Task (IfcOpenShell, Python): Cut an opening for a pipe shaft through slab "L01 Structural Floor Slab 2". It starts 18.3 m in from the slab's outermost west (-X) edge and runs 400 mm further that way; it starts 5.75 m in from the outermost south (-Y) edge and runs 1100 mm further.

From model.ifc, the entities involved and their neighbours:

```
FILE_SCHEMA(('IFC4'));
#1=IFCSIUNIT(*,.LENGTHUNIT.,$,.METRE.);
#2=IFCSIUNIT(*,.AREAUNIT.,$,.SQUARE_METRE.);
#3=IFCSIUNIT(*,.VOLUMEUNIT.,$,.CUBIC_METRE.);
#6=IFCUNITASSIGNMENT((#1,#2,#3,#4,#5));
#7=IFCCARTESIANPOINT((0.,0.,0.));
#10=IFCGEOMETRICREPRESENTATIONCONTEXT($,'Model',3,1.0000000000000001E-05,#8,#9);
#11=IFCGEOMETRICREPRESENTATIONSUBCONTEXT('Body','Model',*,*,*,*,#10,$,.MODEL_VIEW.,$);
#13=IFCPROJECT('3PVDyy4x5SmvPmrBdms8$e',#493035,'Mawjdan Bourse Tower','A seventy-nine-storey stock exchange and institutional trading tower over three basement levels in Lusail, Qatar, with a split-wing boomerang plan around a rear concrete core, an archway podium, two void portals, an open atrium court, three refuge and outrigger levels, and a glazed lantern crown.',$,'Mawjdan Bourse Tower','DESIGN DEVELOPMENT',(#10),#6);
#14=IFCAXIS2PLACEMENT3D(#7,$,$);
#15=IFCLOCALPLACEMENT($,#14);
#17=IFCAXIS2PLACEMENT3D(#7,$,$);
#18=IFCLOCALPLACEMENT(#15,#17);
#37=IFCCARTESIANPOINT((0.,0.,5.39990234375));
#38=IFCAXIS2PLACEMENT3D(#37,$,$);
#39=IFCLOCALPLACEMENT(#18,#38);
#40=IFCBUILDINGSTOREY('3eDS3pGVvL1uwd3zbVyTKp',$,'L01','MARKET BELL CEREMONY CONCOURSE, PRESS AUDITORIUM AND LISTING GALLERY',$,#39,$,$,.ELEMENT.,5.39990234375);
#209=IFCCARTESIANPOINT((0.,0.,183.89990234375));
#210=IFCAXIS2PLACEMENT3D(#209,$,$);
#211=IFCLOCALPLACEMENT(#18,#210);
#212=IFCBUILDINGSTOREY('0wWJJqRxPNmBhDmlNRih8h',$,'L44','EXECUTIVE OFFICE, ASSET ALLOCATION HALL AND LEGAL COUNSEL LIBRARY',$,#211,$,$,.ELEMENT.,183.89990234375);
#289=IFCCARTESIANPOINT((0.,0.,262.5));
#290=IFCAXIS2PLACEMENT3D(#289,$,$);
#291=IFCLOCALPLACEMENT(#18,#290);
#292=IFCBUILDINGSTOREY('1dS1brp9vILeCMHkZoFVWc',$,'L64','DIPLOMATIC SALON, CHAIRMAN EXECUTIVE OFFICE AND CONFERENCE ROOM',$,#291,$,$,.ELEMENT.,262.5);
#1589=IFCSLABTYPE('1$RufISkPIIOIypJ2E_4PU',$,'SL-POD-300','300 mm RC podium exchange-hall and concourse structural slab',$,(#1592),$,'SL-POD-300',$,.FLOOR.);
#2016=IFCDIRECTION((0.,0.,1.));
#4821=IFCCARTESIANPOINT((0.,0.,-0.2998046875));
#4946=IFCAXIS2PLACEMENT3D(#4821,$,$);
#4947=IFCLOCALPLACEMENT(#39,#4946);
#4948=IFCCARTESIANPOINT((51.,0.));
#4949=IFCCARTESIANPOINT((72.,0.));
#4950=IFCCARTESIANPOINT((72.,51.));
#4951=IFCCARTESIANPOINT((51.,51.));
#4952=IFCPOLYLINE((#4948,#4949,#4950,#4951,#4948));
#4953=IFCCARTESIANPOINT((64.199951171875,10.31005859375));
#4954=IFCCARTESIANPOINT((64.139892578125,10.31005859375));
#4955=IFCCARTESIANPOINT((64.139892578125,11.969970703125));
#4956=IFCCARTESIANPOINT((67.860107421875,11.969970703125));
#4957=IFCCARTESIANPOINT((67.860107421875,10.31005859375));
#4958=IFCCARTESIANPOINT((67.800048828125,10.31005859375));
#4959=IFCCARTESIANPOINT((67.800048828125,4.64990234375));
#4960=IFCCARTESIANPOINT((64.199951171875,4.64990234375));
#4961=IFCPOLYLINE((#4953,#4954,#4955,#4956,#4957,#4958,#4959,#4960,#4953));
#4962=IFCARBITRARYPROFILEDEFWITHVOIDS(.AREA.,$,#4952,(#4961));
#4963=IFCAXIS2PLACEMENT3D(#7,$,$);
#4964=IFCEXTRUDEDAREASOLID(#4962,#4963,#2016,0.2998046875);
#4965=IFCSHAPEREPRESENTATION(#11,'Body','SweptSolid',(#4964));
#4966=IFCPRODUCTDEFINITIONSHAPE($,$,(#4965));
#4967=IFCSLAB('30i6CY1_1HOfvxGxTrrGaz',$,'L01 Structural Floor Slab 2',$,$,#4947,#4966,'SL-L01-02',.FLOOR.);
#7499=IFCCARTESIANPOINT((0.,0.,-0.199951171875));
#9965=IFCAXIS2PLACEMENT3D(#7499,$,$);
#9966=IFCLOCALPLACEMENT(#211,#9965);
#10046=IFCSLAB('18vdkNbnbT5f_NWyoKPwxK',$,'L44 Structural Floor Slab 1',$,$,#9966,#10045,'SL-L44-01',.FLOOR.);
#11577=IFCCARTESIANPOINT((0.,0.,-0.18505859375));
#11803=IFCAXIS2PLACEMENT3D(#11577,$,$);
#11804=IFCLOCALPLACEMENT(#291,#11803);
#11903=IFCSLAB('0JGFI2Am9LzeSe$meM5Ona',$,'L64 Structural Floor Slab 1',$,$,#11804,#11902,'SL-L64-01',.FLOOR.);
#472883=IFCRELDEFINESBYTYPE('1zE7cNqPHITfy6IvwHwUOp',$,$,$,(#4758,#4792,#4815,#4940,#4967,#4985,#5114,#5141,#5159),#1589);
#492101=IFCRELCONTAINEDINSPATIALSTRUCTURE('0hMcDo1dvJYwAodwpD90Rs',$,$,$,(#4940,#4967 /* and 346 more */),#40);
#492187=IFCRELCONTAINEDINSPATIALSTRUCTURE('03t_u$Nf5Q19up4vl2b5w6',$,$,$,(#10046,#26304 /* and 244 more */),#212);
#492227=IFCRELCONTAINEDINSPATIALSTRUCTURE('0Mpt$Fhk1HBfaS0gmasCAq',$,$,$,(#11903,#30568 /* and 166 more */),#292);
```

```python
import numpy as np
import ifcopenshell
import ifcopenshell.api.feature
import ifcopenshell.api.geometry
import ifcopenshell.api.root
import ifcopenshell.geom
import ifcopenshell.util.placement
import ifcopenshell.util.representation
import ifcopenshell.util.shape
import ifcopenshell.util.unit

model = ifcopenshell.open("model.ifc")
unit_scale = ifcopenshell.util.unit.calculate_unit_scale(model)
settings = ifcopenshell.geom.settings()


def volume(element):
    """Net volume in cubic metres, openings subtracted."""
    shape = ifcopenshell.geom.create_shape(settings, element)
    return ifcopenshell.util.shape.get_volume(shape.geometry)


slab = model.by_guid("30i6CY1_1HOfvxGxTrrGaz")
before = volume(slab)

# Extent in the slab's own axes, in metres. The edges named are its -X and -Y sides.
slab_shape = ifcopenshell.geom.create_shape(settings, slab)
vertices = ifcopenshell.util.shape.get_vertices(slab_shape.geometry)
x_min, y_min, bottom = vertices.min(axis=0)
top = vertices[:, 2].max()

opening = ifcopenshell.api.root.create_entity(model, ifc_class="IfcOpeningElement", name="Pipe shaft opening", predefined_type="OPENING")
context = ifcopenshell.util.representation.get_context(model, "Model", "Body", "MODEL_VIEW")
width, depth = 0.4, 1.1
outline = [(0.0, 0.0), (width, 0.0), (width, depth), (0.0, depth), (0.0, 0.0)]
# Overshoot both faces by 50 mm so the cut is clean.
shape = ifcopenshell.api.geometry.add_slab_representation(
    model, context=context, depth=top - bottom + 0.1, polyline=outline
)
ifcopenshell.api.geometry.assign_representation(model, product=opening, representation=shape)

matrix = ifcopenshell.util.placement.get_local_placement(slab.ObjectPlacement)
matrix[:, 3] = matrix @ np.append(np.array([x_min + 18.3, y_min + 5.75, bottom - 0.05]) / unit_scale, 1.0)
ifcopenshell.api.geometry.edit_object_placement(model, product=opening, matrix=matrix, is_si=False)
ifcopenshell.api.feature.add_feature(model, feature=opening, element=slab)

after = volume(slab)

print(f"slab volume {before:.3f} -> {after:.3f} m3")

model.write("model_rev.ifc")
```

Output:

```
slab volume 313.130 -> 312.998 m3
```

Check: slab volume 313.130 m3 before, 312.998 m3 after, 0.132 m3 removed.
